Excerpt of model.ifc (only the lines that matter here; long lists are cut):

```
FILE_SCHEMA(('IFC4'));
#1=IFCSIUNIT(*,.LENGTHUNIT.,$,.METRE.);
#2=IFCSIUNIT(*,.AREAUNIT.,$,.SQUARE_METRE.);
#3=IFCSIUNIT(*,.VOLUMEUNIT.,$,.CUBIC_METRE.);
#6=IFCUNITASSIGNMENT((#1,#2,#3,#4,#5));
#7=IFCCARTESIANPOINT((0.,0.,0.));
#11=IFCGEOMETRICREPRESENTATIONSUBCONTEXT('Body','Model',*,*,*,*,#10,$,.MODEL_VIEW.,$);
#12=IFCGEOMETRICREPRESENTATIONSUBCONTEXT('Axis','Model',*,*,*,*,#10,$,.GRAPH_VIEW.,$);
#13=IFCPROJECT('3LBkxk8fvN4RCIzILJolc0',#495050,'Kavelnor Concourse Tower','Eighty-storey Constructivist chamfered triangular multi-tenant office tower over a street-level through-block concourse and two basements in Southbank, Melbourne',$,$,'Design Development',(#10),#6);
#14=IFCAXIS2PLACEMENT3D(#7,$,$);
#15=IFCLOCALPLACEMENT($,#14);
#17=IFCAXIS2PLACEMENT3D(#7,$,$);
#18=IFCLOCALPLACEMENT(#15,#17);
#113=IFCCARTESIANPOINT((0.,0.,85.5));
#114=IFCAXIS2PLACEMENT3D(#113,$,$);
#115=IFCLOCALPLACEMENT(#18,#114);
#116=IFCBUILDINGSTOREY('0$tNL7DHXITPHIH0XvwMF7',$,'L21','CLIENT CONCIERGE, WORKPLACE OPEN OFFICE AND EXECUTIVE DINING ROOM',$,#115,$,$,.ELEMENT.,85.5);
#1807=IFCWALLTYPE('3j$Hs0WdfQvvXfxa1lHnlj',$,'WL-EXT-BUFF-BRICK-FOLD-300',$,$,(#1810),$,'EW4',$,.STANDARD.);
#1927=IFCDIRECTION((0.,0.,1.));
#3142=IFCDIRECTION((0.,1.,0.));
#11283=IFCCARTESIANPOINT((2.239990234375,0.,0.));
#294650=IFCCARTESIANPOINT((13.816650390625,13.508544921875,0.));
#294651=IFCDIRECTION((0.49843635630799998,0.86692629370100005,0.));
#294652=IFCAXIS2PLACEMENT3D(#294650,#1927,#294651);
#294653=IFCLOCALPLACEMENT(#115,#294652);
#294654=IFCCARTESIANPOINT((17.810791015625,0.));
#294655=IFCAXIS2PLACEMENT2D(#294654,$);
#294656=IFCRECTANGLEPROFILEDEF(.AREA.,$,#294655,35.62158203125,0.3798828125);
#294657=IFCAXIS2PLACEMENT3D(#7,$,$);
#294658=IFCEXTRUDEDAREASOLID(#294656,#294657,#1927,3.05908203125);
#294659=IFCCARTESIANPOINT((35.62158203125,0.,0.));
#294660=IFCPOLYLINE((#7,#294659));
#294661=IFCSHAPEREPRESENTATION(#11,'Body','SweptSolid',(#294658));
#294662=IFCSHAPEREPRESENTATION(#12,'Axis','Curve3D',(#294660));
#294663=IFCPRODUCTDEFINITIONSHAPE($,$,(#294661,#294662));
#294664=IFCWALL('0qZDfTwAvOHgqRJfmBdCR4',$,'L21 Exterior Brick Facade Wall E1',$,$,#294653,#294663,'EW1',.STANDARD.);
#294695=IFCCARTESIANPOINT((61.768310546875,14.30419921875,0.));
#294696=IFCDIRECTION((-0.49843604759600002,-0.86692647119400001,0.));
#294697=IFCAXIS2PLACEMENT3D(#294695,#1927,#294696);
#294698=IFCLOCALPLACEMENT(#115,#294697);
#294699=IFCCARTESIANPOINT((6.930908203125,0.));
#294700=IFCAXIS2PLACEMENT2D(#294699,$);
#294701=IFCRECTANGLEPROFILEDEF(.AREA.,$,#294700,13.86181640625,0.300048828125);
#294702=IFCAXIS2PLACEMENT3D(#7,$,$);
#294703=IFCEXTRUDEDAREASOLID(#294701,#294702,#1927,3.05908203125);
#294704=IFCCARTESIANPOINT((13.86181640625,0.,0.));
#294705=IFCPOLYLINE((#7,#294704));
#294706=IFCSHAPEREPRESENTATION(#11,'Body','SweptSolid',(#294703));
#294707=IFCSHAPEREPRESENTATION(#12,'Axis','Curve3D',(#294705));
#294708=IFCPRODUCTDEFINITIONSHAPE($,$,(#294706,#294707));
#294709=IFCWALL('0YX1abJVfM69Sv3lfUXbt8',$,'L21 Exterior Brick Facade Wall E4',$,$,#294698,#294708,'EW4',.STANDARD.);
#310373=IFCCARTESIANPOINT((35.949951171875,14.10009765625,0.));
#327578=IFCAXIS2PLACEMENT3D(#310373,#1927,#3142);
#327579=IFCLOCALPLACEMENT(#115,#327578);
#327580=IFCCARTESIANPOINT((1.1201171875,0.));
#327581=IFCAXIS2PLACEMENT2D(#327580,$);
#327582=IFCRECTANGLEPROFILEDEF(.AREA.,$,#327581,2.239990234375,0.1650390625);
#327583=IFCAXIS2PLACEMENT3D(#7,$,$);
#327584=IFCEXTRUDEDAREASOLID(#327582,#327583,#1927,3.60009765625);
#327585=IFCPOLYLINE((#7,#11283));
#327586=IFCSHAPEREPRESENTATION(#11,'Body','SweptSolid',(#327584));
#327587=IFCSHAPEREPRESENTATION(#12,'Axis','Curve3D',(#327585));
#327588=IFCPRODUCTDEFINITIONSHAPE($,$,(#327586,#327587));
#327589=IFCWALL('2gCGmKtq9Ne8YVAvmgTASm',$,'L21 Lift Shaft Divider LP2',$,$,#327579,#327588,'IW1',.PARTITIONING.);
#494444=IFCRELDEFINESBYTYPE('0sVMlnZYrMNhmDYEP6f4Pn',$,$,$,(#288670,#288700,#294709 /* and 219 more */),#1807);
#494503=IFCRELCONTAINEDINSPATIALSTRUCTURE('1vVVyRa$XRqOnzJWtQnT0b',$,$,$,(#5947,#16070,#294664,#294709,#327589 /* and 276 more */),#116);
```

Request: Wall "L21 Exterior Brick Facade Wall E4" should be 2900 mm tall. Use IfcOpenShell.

```python
import ifcopenshell
import ifcopenshell.geom
import ifcopenshell.util.representation
import ifcopenshell.util.shape
import ifcopenshell.util.unit

model = ifcopenshell.open("model.ifc")
unit_scale = ifcopenshell.util.unit.calculate_unit_scale(model)
settings = ifcopenshell.geom.settings()


def volume(element):
    """Net volume in cubic metres, openings subtracted."""
    shape = ifcopenshell.geom.create_shape(settings, element)
    return ifcopenshell.util.shape.get_volume(shape.geometry)


wall = model.by_guid("0YX1abJVfM69Sv3lfUXbt8")
before = volume(wall)

body = ifcopenshell.util.representation.get_representation(wall, "Model", "Body")
solid = body.Items[0]
old_height = solid.Depth
solid.Depth = 2.9 / unit_scale
after = volume(wall)

print(f"height {old_height:g} -> {solid.Depth:g}, volume {before:.3f} -> {after:.3f} m3")

model.write("model_updated.ifc")
```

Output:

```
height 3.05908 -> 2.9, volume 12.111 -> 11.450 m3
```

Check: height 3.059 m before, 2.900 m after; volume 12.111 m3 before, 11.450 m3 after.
